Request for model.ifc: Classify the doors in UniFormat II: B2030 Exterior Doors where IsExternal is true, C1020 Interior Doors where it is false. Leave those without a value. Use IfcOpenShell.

First a look at what the model holds.

```python
import ifcopenshell
import ifcopenshell.util.element

model = ifcopenshell.open("model.ifc")
print(model.schema)
print("classifications:", [c.Name for c in model.by_type("IfcClassification")])
values = [ifcopenshell.util.element.get_pset(e, "Pset_DoorCommon", "IsExternal") for e in model.by_type("IfcDoor")]
for value in (True, False, None):
    print("IsExternal", value, values.count(value))
```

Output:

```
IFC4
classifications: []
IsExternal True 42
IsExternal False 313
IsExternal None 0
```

```python
import ifcopenshell
import ifcopenshell.api.classification
import ifcopenshell.util.element

model = ifcopenshell.open("model.ifc")

system = ifcopenshell.api.classification.add_classification(model, classification="UniFormat II")

doors = model.by_type("IfcDoor")
external = {e: ifcopenshell.util.element.get_pset(e, "Pset_DoorCommon", "IsExternal") for e in doors}
for flag, code, name in ((True, "B2030", "Exterior Doors"), (False, "C1020", "Interior Doors")):
    products = [e for e in doors if external[e] is flag]
    ifcopenshell.api.classification.add_reference(
        model, products=products, classification=system, identification=code, name=name
    )
    print(code, len(products))

model.write("model_rev.ifc")
```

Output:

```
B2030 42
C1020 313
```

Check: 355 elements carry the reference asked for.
